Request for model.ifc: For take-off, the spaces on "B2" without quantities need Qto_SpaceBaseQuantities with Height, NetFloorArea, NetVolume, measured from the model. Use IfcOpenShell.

First a look at what the model holds.

```python
import ifcopenshell
import ifcopenshell.util.element
import ifcopenshell.util.unit

model = ifcopenshell.open("model.ifc")
print(model.schema)
for unit_type in ("LENGTHUNIT", "AREAUNIT", "VOLUMEUNIT"):
    print(unit_type, ifcopenshell.util.unit.calculate_unit_scale(model, unit_type))
storey = next(s for s in model.by_type("IfcBuildingStorey") if s.Name == "B2")
spaces = [e for e in ifcopenshell.util.element.get_decomposition(storey) if e.is_a("IfcSpace")]
for e in sorted(spaces, key=lambda e: e.id()):
    print(e.id(), e.is_a(), e.Name, list(ifcopenshell.util.element.get_psets(e, qtos_only=True)), sep=" | ")
```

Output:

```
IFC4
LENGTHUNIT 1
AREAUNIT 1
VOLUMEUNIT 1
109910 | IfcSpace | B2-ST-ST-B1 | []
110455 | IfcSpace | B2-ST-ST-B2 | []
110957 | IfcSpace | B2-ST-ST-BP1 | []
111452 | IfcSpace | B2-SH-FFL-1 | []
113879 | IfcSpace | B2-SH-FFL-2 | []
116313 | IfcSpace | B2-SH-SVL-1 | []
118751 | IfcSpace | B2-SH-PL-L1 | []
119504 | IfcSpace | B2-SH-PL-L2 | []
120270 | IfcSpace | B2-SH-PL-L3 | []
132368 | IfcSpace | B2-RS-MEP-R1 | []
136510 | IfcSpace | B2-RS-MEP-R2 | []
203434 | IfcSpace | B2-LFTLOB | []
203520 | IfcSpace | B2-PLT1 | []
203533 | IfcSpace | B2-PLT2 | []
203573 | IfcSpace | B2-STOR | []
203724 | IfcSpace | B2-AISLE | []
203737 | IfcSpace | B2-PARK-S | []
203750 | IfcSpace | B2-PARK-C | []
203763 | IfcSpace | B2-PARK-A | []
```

```python
import ifcopenshell
import ifcopenshell.api.pset
import ifcopenshell.geom
import ifcopenshell.util.element
import ifcopenshell.util.shape
import ifcopenshell.util.unit

model = ifcopenshell.open("model.ifc")
unit_scale = ifcopenshell.util.unit.calculate_unit_scale(model)
area_scale = ifcopenshell.util.unit.calculate_unit_scale(model, "AREAUNIT")
volume_scale = ifcopenshell.util.unit.calculate_unit_scale(model, "VOLUMEUNIT")
settings = ifcopenshell.geom.settings()

storey = next(s for s in model.by_type("IfcBuildingStorey") if s.Name == "B2")
spaces = [e for e in ifcopenshell.util.element.get_decomposition(storey) if e.is_a("IfcSpace")]

for e in sorted(spaces, key=lambda e: e.id()):
    if ifcopenshell.util.element.get_psets(e, qtos_only=True, should_inherit=False):
        continue
    # Geometry comes back in metres, in the element's own axes.
    shape = ifcopenshell.geom.create_shape(settings, e)
    values = {
        "Height": ifcopenshell.util.shape.get_z(shape.geometry) / unit_scale,
        "NetFloorArea": ifcopenshell.util.shape.get_footprint_area(shape.geometry) / area_scale,
        "NetVolume": ifcopenshell.util.shape.get_volume(shape.geometry) / volume_scale,
    }
    qto = ifcopenshell.api.pset.add_qto(model, product=e, name="Qto_SpaceBaseQuantities")
    ifcopenshell.api.pset.edit_qto(model, qto=qto, properties=values)
    print(e.id(), {k: round(v, 3) for k, v in values.items()})

model.write("model_v2.ifc")
```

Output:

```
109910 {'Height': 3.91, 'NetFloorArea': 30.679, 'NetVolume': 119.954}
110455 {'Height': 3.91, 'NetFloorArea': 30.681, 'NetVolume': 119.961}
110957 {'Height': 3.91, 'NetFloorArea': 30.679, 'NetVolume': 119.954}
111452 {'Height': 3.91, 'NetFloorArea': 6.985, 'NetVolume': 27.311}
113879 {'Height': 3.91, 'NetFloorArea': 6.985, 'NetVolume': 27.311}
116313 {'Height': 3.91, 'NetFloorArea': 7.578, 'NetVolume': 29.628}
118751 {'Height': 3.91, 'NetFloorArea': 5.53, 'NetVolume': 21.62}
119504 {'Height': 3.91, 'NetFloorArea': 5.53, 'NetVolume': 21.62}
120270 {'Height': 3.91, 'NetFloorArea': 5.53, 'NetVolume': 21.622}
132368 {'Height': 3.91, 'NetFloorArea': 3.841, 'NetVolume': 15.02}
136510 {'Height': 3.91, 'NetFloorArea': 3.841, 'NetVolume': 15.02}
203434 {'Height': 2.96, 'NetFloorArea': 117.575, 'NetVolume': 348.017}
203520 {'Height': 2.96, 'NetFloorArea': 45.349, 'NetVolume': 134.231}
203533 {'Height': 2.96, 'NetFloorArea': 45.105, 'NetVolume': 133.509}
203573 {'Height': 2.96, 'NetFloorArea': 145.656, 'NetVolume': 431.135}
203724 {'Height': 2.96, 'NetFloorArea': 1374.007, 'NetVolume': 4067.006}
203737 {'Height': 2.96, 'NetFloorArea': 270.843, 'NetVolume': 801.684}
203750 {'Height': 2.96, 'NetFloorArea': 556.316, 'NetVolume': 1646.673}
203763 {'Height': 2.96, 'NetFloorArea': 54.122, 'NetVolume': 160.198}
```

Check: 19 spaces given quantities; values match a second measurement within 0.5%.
